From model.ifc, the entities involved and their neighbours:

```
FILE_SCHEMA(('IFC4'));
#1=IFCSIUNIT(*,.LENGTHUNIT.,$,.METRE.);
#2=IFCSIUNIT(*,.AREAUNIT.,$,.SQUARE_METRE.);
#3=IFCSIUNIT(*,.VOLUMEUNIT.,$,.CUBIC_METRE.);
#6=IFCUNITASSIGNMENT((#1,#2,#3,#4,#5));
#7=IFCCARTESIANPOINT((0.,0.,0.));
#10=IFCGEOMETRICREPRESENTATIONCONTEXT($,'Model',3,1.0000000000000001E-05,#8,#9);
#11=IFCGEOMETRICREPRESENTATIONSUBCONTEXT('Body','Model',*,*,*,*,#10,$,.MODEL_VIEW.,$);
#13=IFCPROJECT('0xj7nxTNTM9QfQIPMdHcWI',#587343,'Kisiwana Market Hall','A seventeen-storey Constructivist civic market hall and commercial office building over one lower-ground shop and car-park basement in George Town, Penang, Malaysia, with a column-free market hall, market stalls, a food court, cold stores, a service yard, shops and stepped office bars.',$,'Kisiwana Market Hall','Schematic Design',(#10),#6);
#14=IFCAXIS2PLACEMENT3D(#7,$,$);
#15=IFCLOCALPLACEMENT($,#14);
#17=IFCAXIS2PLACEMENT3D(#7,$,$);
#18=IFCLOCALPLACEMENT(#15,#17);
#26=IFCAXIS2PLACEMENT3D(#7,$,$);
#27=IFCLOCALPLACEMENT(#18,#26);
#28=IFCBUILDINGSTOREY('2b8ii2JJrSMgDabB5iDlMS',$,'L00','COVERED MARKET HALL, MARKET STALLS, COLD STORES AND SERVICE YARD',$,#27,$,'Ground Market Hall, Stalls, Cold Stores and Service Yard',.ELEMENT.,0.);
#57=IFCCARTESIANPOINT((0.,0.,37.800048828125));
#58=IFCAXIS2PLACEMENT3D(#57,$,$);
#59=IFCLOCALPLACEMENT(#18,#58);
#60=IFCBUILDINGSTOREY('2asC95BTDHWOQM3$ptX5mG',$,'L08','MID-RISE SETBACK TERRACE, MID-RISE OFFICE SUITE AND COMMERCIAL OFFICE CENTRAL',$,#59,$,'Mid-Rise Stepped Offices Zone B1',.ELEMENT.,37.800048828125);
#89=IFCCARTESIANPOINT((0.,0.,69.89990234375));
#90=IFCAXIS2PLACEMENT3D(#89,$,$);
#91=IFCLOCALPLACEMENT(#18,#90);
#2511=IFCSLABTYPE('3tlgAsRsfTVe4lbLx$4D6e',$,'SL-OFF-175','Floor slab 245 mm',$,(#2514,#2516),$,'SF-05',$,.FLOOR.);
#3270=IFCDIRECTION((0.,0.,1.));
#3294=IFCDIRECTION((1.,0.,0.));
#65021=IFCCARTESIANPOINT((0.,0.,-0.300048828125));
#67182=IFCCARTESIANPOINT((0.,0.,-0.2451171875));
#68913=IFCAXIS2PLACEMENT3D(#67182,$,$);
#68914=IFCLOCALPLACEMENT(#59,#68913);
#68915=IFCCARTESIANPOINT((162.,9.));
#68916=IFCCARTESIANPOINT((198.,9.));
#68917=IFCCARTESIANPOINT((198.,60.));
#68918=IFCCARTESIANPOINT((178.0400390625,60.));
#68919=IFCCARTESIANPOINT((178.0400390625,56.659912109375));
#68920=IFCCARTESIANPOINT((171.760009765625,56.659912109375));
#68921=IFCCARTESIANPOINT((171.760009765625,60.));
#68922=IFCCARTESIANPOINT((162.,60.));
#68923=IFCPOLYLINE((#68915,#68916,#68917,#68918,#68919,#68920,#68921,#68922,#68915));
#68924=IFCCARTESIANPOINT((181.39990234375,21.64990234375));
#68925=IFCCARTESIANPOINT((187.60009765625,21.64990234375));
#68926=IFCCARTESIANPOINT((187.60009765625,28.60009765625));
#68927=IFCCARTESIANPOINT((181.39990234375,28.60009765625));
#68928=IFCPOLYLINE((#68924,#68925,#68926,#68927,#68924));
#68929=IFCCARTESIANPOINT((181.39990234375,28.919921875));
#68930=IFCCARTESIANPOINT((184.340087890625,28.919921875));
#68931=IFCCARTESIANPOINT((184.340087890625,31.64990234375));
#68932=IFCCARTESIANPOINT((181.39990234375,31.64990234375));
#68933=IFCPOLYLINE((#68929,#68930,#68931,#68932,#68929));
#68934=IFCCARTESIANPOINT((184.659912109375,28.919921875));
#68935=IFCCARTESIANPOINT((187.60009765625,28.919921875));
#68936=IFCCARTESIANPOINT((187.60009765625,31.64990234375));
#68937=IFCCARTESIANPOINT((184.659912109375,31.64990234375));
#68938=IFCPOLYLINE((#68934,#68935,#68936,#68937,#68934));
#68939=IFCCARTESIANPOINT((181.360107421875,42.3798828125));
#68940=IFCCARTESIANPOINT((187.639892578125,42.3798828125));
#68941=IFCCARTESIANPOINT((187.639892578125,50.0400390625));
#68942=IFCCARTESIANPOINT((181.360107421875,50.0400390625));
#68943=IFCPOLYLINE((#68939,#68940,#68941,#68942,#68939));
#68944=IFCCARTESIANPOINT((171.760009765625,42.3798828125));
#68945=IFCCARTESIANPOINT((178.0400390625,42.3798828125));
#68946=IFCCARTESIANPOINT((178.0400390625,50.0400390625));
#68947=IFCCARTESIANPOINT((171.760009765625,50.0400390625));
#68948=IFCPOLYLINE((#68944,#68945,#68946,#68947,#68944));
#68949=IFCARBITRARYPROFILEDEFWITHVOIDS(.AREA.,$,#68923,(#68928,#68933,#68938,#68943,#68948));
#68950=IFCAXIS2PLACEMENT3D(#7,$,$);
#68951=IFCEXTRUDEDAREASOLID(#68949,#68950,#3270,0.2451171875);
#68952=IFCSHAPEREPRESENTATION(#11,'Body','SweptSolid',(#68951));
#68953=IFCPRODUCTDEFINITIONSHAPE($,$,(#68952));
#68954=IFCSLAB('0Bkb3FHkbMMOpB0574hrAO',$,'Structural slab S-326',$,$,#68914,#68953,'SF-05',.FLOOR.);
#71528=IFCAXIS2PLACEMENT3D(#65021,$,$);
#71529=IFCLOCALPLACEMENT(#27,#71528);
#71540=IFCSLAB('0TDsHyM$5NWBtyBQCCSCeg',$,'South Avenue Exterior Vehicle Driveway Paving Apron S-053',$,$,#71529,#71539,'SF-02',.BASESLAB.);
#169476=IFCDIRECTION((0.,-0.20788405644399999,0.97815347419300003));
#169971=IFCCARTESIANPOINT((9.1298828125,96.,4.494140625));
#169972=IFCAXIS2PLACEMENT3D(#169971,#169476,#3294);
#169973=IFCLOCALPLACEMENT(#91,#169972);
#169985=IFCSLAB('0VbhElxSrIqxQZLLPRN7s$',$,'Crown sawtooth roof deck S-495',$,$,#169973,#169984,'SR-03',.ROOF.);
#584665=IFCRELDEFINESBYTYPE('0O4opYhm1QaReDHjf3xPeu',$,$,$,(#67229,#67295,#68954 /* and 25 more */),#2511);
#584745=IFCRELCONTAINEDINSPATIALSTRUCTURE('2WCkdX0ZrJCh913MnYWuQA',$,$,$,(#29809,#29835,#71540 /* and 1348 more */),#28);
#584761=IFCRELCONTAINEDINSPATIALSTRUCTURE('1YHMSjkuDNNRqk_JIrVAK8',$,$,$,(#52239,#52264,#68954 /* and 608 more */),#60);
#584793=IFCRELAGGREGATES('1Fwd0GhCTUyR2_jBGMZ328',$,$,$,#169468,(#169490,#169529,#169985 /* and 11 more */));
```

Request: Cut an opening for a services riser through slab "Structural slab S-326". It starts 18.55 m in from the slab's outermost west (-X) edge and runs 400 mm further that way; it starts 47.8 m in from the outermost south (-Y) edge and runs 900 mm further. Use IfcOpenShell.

```python
import numpy as np
import ifcopenshell
import ifcopenshell.api.feature
import ifcopenshell.api.geometry
import ifcopenshell.api.root
import ifcopenshell.geom
import ifcopenshell.util.placement
import ifcopenshell.util.representation
import ifcopenshell.util.shape
import ifcopenshell.util.unit

model = ifcopenshell.open("model.ifc")
unit_scale = ifcopenshell.util.unit.calculate_unit_scale(model)
settings = ifcopenshell.geom.settings()


def volume(element):
    """Net volume in cubic metres, openings subtracted."""
    shape = ifcopenshell.geom.create_shape(settings, element)
    return ifcopenshell.util.shape.get_volume(shape.geometry)


slab = model.by_id(68954)
before = volume(slab)

# Extent in the slab's own axes, in metres. The edges named are its -X and -Y sides.
slab_shape = ifcopenshell.geom.create_shape(settings, slab)
vertices = ifcopenshell.util.shape.get_vertices(slab_shape.geometry)
x_min, y_min, bottom = vertices.min(axis=0)
top = vertices[:, 2].max()

opening = ifcopenshell.api.root.create_entity(model, ifc_class="IfcOpeningElement", name="Services riser opening", predefined_type="OPENING")
context = ifcopenshell.util.representation.get_context(model, "Model", "Body", "MODEL_VIEW")
width, depth = 0.4, 0.9
outline = [(0.0, 0.0), (width, 0.0), (width, depth), (0.0, depth), (0.0, 0.0)]
# Overshoot both faces by 50 mm so the cut is clean.
shape = ifcopenshell.api.geometry.add_slab_representation(
    model, context=context, depth=top - bottom + 0.1, polyline=outline
)
ifcopenshell.api.geometry.assign_representation(model, product=opening, representation=shape)

matrix = ifcopenshell.util.placement.get_local_placement(slab.ObjectPlacement)
matrix[:, 3] = matrix @ np.append(np.array([x_min + 18.55, y_min + 47.8, bottom - 0.05]) / unit_scale, 1.0)
ifcopenshell.api.geometry.edit_object_placement(model, product=opening, matrix=matrix, is_si=False)
ifcopenshell.api.feature.add_feature(model, feature=opening, element=slab)

after = volume(slab)

print(f"slab volume {before:.3f} -> {after:.3f} m3")

model.write("model-out.ifc")
```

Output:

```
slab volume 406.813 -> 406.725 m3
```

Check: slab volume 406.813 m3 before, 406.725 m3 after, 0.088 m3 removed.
